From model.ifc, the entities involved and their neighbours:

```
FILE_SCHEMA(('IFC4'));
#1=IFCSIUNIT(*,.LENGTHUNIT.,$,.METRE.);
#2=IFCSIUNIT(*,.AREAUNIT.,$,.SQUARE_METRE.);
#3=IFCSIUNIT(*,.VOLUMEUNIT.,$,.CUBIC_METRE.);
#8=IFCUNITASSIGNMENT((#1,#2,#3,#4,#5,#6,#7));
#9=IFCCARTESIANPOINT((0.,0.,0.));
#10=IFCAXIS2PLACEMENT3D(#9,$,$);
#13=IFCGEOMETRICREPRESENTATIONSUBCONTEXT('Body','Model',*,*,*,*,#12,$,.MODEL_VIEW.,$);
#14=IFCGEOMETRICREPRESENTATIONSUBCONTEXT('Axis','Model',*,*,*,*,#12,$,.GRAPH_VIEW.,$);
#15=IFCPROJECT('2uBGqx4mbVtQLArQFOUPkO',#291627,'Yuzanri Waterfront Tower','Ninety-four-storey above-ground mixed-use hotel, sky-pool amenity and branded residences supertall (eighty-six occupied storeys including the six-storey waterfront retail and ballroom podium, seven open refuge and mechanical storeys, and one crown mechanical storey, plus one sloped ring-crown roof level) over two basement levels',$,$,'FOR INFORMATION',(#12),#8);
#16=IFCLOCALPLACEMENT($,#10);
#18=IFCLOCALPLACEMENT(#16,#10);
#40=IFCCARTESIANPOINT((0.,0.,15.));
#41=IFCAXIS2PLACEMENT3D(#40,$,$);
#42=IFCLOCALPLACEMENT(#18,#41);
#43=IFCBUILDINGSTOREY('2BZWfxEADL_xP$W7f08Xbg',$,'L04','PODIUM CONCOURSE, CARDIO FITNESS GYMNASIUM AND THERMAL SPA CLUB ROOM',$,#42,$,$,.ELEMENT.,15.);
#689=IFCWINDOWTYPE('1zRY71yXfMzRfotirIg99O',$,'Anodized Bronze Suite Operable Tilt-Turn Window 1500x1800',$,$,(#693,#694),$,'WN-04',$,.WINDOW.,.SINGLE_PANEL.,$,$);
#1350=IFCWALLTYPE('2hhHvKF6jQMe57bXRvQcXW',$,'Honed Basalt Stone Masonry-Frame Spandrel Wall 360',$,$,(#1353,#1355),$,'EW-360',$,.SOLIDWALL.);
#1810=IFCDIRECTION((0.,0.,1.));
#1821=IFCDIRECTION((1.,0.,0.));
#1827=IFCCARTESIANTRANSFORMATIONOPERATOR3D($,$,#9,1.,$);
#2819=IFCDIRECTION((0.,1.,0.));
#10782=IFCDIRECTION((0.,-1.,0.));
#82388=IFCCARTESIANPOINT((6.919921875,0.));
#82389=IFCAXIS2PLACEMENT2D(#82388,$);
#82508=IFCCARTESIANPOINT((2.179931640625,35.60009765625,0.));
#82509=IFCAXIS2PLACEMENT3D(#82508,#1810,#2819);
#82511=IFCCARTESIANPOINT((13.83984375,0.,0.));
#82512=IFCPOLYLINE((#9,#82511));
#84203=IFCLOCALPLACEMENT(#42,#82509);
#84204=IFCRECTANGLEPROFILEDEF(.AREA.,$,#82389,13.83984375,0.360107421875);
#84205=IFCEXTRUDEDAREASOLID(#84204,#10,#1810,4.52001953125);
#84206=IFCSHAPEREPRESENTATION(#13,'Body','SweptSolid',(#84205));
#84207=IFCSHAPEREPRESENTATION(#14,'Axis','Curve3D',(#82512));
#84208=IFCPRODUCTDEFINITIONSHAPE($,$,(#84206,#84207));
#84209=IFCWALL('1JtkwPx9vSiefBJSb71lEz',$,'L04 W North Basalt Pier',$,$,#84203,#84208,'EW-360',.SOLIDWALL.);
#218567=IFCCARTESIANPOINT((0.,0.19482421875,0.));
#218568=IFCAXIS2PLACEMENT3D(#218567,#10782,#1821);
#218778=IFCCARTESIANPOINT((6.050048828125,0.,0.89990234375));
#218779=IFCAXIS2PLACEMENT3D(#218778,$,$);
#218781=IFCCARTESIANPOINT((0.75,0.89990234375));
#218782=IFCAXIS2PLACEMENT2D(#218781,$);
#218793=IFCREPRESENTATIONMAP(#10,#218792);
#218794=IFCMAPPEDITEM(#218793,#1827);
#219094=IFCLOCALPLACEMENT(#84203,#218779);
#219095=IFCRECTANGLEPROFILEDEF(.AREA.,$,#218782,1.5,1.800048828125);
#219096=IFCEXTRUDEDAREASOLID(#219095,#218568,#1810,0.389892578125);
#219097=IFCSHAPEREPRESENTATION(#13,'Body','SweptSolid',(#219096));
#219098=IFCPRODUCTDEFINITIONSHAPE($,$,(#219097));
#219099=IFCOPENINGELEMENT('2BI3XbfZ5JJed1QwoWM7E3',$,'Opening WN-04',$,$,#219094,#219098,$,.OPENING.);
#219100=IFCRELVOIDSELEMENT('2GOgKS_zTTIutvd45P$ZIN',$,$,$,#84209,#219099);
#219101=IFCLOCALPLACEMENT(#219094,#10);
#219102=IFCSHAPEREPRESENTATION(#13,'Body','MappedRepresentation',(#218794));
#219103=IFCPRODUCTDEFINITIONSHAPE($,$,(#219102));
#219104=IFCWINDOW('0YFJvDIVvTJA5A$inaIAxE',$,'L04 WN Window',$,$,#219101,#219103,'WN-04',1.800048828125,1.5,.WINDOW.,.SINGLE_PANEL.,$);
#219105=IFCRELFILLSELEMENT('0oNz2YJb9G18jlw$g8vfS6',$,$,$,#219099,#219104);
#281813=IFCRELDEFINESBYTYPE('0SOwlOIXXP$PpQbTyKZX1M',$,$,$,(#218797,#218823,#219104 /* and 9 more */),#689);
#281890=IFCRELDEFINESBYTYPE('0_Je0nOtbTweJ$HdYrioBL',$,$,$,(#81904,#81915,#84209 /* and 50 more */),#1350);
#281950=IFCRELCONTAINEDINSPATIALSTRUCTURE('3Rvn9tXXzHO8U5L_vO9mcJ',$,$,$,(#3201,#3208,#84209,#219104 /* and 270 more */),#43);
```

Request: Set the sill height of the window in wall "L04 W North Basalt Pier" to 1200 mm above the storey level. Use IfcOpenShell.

```python
import numpy as np
import ifcopenshell
import ifcopenshell.api.geometry
import ifcopenshell.geom
import ifcopenshell.util.element
import ifcopenshell.util.placement
import ifcopenshell.util.shape
import ifcopenshell.util.unit

model = ifcopenshell.open("model.ifc")
unit_scale = ifcopenshell.util.unit.calculate_unit_scale(model)

window = model.by_guid("0YFJvDIVvTJA5A$inaIAxE")
opening = window.FillsVoids[0].RelatingOpeningElement
storey = ifcopenshell.util.element.get_container(window, ifc_class="IfcBuildingStorey")
level = ifcopenshell.util.placement.get_local_placement(storey.ObjectPlacement)[2, 3]

# The opening's origin need not be at the sill, so measure its lowest point.
shape = ifcopenshell.geom.create_shape(ifcopenshell.geom.settings(), opening)
bottom = ifcopenshell.util.shape.get_shape_bottom_elevation(shape, shape.geometry) / unit_scale
dz = level + 1.2 / unit_scale - bottom

shift = np.array([0.0, 0.0, dz])
# The window is placed relative to its opening, so it follows when the opening moves.
matrix = ifcopenshell.util.placement.get_local_placement(opening.ObjectPlacement)
matrix[:3, 3] += shift
ifcopenshell.api.geometry.edit_object_placement(
    model, product=opening, matrix=matrix, is_si=False, should_transform_children=True
)

print(f"moved by {dz * unit_scale:+.3f} m")

model.write("model_updated.ifc")
```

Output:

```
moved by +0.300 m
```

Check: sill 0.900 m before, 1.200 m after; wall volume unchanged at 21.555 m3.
